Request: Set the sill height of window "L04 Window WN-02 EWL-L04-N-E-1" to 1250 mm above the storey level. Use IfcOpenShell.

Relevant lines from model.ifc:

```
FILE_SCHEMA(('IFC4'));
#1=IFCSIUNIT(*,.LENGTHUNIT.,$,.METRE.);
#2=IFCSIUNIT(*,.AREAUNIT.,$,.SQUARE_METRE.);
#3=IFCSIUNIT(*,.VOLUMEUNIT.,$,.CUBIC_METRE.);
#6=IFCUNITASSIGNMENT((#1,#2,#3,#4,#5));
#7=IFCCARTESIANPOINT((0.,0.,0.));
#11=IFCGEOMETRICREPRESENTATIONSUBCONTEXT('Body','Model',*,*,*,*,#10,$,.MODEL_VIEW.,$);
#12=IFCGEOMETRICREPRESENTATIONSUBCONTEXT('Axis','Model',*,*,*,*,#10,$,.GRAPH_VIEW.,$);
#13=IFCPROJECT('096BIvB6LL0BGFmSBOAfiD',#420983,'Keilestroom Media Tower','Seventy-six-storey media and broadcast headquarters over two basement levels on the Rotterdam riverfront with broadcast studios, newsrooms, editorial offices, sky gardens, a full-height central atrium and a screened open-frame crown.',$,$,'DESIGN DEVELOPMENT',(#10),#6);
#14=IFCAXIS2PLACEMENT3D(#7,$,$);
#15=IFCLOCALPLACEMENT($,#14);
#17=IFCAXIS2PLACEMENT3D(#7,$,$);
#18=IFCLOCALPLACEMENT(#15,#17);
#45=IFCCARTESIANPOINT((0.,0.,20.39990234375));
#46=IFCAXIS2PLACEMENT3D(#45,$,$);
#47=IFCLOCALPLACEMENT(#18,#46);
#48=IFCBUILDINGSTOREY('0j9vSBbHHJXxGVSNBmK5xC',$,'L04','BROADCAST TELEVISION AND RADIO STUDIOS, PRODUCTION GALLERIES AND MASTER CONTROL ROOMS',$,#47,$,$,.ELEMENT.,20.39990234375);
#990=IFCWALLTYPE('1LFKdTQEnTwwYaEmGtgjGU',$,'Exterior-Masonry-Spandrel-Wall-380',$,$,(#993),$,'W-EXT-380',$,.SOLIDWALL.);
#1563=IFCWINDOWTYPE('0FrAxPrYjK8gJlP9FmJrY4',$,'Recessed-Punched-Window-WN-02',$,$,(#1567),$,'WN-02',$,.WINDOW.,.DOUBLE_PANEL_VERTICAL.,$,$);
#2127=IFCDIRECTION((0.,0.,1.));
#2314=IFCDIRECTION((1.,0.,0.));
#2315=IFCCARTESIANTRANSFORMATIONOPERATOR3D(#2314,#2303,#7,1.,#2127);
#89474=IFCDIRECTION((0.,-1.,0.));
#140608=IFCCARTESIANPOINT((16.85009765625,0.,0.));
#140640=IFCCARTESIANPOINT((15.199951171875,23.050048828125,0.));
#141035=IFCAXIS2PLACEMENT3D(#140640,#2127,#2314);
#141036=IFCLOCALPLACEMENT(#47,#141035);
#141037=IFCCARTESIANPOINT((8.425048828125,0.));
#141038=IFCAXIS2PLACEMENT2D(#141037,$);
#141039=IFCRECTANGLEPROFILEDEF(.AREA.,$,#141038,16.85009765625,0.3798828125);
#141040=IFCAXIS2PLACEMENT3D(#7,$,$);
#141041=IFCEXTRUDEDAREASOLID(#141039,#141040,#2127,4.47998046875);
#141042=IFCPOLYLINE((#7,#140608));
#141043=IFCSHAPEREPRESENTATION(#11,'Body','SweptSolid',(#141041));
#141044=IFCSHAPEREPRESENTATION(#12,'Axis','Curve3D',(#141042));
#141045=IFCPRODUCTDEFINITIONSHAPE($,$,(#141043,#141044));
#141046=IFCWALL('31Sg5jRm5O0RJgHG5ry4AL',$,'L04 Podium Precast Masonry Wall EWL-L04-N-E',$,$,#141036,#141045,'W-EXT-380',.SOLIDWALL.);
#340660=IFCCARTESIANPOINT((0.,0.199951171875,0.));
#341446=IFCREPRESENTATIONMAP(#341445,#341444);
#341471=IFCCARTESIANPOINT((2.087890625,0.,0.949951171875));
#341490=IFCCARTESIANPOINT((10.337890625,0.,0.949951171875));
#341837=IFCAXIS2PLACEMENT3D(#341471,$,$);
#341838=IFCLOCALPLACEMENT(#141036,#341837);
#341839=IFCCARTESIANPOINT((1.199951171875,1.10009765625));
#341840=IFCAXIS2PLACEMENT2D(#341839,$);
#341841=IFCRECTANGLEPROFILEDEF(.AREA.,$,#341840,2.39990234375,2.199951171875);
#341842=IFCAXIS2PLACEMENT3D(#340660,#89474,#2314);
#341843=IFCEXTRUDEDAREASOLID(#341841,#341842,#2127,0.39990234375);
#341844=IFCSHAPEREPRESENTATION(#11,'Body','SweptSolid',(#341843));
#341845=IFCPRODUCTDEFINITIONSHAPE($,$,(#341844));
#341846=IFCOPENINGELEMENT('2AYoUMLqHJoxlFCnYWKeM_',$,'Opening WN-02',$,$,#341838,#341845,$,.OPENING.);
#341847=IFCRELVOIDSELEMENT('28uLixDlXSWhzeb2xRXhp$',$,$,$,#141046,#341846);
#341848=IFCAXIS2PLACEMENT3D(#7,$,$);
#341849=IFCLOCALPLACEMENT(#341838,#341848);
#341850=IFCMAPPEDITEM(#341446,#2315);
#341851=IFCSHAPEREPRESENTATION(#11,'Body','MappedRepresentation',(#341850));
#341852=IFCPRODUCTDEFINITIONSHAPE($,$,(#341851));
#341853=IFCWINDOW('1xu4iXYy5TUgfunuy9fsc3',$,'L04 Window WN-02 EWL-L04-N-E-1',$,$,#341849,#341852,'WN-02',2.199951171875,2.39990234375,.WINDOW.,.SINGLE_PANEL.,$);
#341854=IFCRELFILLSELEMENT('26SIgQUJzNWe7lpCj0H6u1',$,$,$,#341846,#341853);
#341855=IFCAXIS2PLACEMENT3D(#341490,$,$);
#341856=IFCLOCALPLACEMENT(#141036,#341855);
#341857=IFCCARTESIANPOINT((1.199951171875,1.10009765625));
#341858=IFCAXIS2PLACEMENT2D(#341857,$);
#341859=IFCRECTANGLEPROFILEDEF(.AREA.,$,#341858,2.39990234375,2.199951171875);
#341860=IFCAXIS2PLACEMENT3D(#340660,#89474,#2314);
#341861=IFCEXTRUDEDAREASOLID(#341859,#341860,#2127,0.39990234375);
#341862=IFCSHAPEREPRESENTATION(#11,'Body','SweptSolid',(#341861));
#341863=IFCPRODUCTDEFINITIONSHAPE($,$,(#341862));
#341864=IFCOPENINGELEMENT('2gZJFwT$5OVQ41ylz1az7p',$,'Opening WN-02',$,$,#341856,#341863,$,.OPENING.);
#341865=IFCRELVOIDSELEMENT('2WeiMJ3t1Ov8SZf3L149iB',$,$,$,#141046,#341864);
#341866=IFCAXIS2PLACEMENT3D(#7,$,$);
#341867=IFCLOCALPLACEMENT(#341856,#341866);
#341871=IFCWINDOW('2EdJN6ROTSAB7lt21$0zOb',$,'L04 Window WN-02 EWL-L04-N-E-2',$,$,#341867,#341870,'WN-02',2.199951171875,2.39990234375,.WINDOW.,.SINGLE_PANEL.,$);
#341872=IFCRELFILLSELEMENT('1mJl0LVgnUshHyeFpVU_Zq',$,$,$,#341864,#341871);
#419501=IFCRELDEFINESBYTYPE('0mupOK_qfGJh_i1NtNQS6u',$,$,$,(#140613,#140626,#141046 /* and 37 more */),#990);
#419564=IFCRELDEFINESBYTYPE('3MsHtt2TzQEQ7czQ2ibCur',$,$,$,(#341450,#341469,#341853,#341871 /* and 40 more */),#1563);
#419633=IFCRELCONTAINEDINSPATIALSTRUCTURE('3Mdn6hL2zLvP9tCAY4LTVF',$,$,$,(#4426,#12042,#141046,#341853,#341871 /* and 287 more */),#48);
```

```python
import numpy as np
import ifcopenshell
import ifcopenshell.api.geometry
import ifcopenshell.geom
import ifcopenshell.util.element
import ifcopenshell.util.placement
import ifcopenshell.util.shape
import ifcopenshell.util.unit

model = ifcopenshell.open("model.ifc")
unit_scale = ifcopenshell.util.unit.calculate_unit_scale(model)

window = model.by_guid("1xu4iXYy5TUgfunuy9fsc3")
opening = window.FillsVoids[0].RelatingOpeningElement
storey = ifcopenshell.util.element.get_container(window, ifc_class="IfcBuildingStorey")
level = ifcopenshell.util.placement.get_local_placement(storey.ObjectPlacement)[2, 3]

# The opening's origin need not be at the sill, so measure its lowest point.
shape = ifcopenshell.geom.create_shape(ifcopenshell.geom.settings(), opening)
bottom = ifcopenshell.util.shape.get_shape_bottom_elevation(shape, shape.geometry) / unit_scale
dz = level + 1.25 / unit_scale - bottom

shift = np.array([0.0, 0.0, dz])
# The window is placed relative to its opening, so it follows when the opening moves.
matrix = ifcopenshell.util.placement.get_local_placement(opening.ObjectPlacement)
matrix[:3, 3] += shift
ifcopenshell.api.geometry.edit_object_placement(
    model, product=opening, matrix=matrix, is_si=False, should_transform_children=True
)

print(f"moved by {dz * unit_scale:+.3f} m")

model.write("model_rev.ifc")
```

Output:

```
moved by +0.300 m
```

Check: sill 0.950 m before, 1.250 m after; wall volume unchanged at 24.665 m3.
